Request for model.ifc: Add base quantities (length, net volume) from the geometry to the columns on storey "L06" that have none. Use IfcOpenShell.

First a look at what the model holds.

```python
import ifcopenshell
import ifcopenshell.util.element
import ifcopenshell.util.unit

model = ifcopenshell.open("model.ifc")
print(model.schema)
for unit_type in ("LENGTHUNIT", "AREAUNIT", "VOLUMEUNIT"):
    print(unit_type, ifcopenshell.util.unit.calculate_unit_scale(model, unit_type))
storey = next(s for s in model.by_type("IfcBuildingStorey") if s.Name == "L06")
columns = [e for e in ifcopenshell.util.element.get_decomposition(storey) if e.is_a("IfcColumn")]
for e in sorted(columns, key=lambda e: e.id()):
    print(e.id(), e.is_a(), e.Name, list(ifcopenshell.util.element.get_psets(e, qtos_only=True)), sep=" | ")
```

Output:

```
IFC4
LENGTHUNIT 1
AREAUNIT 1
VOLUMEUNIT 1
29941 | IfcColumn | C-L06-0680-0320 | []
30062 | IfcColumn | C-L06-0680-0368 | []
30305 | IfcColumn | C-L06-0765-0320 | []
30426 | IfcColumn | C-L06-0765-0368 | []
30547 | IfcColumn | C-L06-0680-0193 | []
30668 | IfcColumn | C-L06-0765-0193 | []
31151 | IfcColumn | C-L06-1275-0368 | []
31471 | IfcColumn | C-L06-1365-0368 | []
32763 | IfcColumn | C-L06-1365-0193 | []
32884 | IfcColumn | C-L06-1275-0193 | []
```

```python
import ifcopenshell
import ifcopenshell.api.pset
import ifcopenshell.geom
import ifcopenshell.util.element
import ifcopenshell.util.shape
import ifcopenshell.util.unit

model = ifcopenshell.open("model.ifc")
unit_scale = ifcopenshell.util.unit.calculate_unit_scale(model)
volume_scale = ifcopenshell.util.unit.calculate_unit_scale(model, "VOLUMEUNIT")
settings = ifcopenshell.geom.settings()

storey = next(s for s in model.by_type("IfcBuildingStorey") if s.Name == "L06")
columns = [e for e in ifcopenshell.util.element.get_decomposition(storey) if e.is_a("IfcColumn")]

for e in sorted(columns, key=lambda e: e.id()):
    if ifcopenshell.util.element.get_psets(e, qtos_only=True, should_inherit=False):
        continue
    # Geometry comes back in metres, in the element's own axes.
    shape = ifcopenshell.geom.create_shape(settings, e)
    values = {
        "Length": ifcopenshell.util.shape.get_z(shape.geometry) / unit_scale,
        "NetVolume": ifcopenshell.util.shape.get_volume(shape.geometry) / volume_scale,
    }
    qto = ifcopenshell.api.pset.add_qto(model, product=e, name="Qto_ColumnBaseQuantities")
    ifcopenshell.api.pset.edit_qto(model, qto=qto, properties=values)
    print(e.id(), {k: round(v, 3) for k, v in values.items()})

model.write("model_rev.ifc")
```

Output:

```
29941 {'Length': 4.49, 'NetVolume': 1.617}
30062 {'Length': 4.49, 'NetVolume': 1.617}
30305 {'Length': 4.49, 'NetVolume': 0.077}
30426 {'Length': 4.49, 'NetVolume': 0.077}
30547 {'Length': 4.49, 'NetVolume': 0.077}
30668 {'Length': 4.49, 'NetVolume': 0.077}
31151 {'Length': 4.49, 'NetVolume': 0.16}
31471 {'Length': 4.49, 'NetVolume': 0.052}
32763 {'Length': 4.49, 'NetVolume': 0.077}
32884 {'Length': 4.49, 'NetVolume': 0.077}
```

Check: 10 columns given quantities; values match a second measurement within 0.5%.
